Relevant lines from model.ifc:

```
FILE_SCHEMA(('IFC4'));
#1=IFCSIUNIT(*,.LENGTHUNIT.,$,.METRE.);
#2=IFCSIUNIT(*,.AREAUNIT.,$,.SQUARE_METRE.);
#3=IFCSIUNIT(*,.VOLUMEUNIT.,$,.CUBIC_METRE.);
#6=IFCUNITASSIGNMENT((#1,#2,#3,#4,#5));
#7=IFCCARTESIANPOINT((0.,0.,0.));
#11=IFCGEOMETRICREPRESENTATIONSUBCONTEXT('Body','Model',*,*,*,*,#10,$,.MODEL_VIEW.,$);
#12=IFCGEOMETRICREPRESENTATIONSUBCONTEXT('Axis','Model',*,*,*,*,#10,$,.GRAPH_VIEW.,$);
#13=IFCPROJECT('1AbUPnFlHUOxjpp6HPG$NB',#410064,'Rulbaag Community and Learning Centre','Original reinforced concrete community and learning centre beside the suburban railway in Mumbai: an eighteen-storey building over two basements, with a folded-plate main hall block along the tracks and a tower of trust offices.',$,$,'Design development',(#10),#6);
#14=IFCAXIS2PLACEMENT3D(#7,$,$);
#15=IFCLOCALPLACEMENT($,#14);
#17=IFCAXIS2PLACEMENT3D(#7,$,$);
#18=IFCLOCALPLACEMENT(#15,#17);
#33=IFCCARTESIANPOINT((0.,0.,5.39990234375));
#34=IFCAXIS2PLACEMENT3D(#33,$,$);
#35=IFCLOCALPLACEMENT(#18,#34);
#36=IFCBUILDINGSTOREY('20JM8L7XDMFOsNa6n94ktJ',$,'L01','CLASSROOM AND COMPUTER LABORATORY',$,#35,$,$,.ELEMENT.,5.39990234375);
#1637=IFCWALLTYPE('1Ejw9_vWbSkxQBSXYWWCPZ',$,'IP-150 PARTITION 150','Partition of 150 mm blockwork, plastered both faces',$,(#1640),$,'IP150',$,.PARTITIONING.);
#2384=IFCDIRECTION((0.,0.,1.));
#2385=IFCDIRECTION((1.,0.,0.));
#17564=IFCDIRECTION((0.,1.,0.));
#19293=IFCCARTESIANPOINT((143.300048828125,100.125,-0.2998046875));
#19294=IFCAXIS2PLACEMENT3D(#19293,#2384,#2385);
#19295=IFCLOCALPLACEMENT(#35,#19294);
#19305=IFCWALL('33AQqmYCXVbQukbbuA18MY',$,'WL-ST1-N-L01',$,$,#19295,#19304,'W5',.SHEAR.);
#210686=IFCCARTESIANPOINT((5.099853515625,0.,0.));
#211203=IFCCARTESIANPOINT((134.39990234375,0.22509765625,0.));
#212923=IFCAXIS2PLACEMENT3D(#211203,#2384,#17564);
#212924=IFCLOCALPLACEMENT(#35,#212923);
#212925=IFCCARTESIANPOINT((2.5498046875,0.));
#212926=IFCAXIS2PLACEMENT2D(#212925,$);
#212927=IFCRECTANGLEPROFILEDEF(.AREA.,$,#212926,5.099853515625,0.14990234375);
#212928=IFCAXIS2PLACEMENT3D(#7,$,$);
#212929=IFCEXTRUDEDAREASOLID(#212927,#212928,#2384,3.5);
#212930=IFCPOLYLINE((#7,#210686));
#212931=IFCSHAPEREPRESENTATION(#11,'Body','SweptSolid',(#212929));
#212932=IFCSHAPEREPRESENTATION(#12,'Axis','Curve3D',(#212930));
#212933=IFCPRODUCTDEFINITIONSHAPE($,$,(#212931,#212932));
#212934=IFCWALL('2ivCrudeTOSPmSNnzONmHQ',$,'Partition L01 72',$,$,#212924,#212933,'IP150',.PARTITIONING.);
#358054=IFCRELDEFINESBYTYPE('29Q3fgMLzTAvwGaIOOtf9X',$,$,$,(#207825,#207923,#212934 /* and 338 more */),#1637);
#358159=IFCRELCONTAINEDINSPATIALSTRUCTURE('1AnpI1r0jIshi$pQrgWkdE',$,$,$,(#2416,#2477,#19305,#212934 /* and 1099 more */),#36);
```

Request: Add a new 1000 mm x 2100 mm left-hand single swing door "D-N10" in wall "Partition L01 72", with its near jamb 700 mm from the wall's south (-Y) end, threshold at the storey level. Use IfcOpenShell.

```python
import numpy as np
import ifcopenshell
import ifcopenshell.api.feature
import ifcopenshell.api.geometry
import ifcopenshell.api.root
import ifcopenshell.api.spatial
import ifcopenshell.geom
import ifcopenshell.util.element
import ifcopenshell.util.placement
import ifcopenshell.util.representation
import ifcopenshell.util.shape
import ifcopenshell.util.unit

model = ifcopenshell.open("model.ifc")
unit_scale = ifcopenshell.util.unit.calculate_unit_scale(model)
settings = ifcopenshell.geom.settings()


def volume(element):
    """Net volume in cubic metres, openings subtracted."""
    shape = ifcopenshell.geom.create_shape(settings, element)
    return ifcopenshell.util.shape.get_volume(shape.geometry)


wall = model.by_id(212934)
storey = ifcopenshell.util.element.get_container(wall, ifc_class="IfcBuildingStorey")
context = ifcopenshell.util.representation.get_context(model, "Model", "Body", "MODEL_VIEW")
before = volume(wall)

width, height, from_end, sill = 1, 2.1, 0.7, 0.0  # metres

# The wall runs along its own X axis, and the end named is its -X end.
wall_shape = ifcopenshell.geom.create_shape(settings, wall)
x, y, z = ifcopenshell.util.shape.get_vertices(wall_shape.geometry).T
start = x.min() + from_end
face, thickness = float(y.min()), float(y.max() - y.min())
wall_matrix = ifcopenshell.util.placement.get_local_placement(wall.ObjectPlacement)
level = ifcopenshell.util.placement.get_local_placement(storey.ObjectPlacement)[2, 3]


def in_wall(x, y):
    """Placement at x, y metres in the wall's axes, at sill height."""
    matrix = wall_matrix.copy()
    matrix[:, 3] = wall_matrix @ np.array([x / unit_scale, y / unit_scale, 0.0, 1.0])
    matrix[2, 3] = level + sill / unit_scale
    return matrix


# Opening: a box that overshoots both wall faces by 50 mm.
opening = ifcopenshell.api.root.create_entity(model, ifc_class="IfcOpeningElement", predefined_type="OPENING")
box = ifcopenshell.api.geometry.add_wall_representation(
    model, context=context, length=width, height=height, thickness=thickness + 0.1
)
ifcopenshell.api.geometry.assign_representation(model, product=opening, representation=box)
ifcopenshell.api.geometry.edit_object_placement(model, product=opening, matrix=in_wall(start, face - 0.05), is_si=False)
ifcopenshell.api.feature.add_feature(model, feature=opening, element=wall)

door = ifcopenshell.api.root.create_entity(model, ifc_class="IfcDoor", name="D-N10", predefined_type="DOOR")
door.OverallWidth, door.OverallHeight = width / unit_scale, height / unit_scale
door.OperationType = "SINGLE_SWING_LEFT"
body = ifcopenshell.api.geometry.add_door_representation(
    model,
    context=context,
    overall_width=door.OverallWidth,
    overall_height=door.OverallHeight,
    operation_type="SINGLE_SWING_LEFT",
    lining_properties={"LiningDepth": thickness / unit_scale, "ThresholdDepth": thickness / unit_scale},
)
ifcopenshell.api.geometry.assign_representation(model, product=door, representation=body)
ifcopenshell.api.spatial.assign_container(model, products=[door], relating_structure=storey)
ifcopenshell.api.feature.add_filling(model, opening=opening, element=door)

# The lining spans the wall, so the door starts at the wall face.
ifcopenshell.api.geometry.edit_object_placement(model, product=door, matrix=in_wall(start, face), is_si=False)

after = volume(wall)

print(f"wall volume {before:.3f} -> {after:.3f} m3")

model.write("model-out.ifc")
```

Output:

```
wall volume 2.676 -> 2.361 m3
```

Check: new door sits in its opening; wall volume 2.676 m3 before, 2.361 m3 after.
